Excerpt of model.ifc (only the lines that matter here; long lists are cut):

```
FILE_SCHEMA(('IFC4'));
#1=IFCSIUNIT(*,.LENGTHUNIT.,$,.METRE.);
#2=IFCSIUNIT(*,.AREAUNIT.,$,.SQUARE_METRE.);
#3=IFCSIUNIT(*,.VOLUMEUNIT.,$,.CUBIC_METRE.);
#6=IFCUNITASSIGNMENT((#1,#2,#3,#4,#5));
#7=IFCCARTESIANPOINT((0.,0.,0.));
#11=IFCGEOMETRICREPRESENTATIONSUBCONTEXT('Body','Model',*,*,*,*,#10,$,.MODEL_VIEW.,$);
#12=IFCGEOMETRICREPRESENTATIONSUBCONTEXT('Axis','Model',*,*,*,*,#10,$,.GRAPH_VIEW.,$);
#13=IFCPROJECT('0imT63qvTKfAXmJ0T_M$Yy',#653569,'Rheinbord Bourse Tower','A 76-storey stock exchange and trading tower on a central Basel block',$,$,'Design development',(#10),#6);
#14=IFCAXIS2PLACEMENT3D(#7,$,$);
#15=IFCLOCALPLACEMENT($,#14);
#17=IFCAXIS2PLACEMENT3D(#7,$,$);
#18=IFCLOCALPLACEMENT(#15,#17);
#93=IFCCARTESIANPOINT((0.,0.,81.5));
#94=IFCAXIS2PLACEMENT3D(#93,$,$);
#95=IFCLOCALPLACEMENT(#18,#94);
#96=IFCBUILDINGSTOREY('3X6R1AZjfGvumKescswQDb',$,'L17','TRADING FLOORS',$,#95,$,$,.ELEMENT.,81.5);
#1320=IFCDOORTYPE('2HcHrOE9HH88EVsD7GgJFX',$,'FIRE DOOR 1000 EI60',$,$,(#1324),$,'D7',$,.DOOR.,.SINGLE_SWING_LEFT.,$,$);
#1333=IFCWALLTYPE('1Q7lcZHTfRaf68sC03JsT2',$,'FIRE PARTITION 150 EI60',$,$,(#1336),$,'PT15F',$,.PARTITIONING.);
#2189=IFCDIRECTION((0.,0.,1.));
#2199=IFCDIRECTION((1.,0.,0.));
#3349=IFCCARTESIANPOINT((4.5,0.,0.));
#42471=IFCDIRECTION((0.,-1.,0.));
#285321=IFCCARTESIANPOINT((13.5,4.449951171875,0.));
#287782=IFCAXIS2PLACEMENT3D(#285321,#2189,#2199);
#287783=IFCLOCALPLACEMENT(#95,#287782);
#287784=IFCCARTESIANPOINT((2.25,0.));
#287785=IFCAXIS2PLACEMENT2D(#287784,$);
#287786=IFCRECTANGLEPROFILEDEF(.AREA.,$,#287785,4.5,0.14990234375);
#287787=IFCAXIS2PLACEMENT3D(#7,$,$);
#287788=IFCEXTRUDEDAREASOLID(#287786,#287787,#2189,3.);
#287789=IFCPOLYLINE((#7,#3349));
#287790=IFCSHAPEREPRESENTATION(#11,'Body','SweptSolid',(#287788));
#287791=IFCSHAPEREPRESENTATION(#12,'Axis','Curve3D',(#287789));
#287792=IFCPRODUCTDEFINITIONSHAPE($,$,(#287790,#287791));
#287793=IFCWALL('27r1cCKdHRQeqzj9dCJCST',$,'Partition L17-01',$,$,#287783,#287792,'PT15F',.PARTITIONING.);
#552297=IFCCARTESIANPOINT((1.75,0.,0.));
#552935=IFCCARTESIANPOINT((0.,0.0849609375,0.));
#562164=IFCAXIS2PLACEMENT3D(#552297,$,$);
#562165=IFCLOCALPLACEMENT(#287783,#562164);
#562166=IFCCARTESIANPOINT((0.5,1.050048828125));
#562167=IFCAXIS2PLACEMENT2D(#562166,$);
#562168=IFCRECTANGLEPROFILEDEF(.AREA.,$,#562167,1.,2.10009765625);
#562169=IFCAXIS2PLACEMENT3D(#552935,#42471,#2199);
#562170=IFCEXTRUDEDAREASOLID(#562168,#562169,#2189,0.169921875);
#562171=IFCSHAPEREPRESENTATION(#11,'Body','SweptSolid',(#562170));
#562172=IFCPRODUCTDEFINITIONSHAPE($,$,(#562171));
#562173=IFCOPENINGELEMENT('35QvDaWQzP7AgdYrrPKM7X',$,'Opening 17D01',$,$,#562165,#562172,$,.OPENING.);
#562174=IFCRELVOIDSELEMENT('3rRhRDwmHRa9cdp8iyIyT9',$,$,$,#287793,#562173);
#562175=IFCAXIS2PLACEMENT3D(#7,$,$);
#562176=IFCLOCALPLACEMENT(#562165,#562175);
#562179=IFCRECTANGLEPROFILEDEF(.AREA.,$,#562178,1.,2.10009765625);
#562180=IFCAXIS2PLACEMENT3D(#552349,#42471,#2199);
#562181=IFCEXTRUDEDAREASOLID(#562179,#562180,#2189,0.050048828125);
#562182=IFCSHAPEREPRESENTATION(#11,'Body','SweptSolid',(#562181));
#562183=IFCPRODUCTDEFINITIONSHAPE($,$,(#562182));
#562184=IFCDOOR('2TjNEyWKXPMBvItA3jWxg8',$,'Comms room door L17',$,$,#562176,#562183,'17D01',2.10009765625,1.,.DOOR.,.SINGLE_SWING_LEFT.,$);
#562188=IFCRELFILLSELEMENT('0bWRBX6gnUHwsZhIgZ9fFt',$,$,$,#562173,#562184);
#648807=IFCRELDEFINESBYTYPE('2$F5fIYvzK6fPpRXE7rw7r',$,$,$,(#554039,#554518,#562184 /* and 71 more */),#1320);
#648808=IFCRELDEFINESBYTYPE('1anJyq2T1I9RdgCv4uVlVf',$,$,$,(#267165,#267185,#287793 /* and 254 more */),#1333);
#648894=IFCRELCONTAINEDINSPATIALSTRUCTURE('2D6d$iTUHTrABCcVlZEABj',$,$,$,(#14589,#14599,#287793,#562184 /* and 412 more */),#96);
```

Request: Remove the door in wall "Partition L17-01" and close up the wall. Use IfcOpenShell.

```python
import ifcopenshell
import ifcopenshell.api.feature
import ifcopenshell.api.root
import ifcopenshell.geom
import ifcopenshell.util.shape

model = ifcopenshell.open("model.ifc")
settings = ifcopenshell.geom.settings()


def volume(element):
    """Net volume in cubic metres, openings subtracted."""
    shape = ifcopenshell.geom.create_shape(settings, element)
    return ifcopenshell.util.shape.get_volume(shape.geometry)


door = model.by_guid("2TjNEyWKXPMBvItA3jWxg8")
opening = door.FillsVoids[0].RelatingOpeningElement
wall = opening.VoidsElements[0].RelatingBuildingElement
before = volume(wall)

ifcopenshell.api.root.remove_product(model, product=door)
ifcopenshell.api.feature.remove_feature(model, feature=opening)

after = volume(wall)

print(f"wall volume {before:.3f} -> {after:.3f} m3")

model.write("model_v2.ifc")
```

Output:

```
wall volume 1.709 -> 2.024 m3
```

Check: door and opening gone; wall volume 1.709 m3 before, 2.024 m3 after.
